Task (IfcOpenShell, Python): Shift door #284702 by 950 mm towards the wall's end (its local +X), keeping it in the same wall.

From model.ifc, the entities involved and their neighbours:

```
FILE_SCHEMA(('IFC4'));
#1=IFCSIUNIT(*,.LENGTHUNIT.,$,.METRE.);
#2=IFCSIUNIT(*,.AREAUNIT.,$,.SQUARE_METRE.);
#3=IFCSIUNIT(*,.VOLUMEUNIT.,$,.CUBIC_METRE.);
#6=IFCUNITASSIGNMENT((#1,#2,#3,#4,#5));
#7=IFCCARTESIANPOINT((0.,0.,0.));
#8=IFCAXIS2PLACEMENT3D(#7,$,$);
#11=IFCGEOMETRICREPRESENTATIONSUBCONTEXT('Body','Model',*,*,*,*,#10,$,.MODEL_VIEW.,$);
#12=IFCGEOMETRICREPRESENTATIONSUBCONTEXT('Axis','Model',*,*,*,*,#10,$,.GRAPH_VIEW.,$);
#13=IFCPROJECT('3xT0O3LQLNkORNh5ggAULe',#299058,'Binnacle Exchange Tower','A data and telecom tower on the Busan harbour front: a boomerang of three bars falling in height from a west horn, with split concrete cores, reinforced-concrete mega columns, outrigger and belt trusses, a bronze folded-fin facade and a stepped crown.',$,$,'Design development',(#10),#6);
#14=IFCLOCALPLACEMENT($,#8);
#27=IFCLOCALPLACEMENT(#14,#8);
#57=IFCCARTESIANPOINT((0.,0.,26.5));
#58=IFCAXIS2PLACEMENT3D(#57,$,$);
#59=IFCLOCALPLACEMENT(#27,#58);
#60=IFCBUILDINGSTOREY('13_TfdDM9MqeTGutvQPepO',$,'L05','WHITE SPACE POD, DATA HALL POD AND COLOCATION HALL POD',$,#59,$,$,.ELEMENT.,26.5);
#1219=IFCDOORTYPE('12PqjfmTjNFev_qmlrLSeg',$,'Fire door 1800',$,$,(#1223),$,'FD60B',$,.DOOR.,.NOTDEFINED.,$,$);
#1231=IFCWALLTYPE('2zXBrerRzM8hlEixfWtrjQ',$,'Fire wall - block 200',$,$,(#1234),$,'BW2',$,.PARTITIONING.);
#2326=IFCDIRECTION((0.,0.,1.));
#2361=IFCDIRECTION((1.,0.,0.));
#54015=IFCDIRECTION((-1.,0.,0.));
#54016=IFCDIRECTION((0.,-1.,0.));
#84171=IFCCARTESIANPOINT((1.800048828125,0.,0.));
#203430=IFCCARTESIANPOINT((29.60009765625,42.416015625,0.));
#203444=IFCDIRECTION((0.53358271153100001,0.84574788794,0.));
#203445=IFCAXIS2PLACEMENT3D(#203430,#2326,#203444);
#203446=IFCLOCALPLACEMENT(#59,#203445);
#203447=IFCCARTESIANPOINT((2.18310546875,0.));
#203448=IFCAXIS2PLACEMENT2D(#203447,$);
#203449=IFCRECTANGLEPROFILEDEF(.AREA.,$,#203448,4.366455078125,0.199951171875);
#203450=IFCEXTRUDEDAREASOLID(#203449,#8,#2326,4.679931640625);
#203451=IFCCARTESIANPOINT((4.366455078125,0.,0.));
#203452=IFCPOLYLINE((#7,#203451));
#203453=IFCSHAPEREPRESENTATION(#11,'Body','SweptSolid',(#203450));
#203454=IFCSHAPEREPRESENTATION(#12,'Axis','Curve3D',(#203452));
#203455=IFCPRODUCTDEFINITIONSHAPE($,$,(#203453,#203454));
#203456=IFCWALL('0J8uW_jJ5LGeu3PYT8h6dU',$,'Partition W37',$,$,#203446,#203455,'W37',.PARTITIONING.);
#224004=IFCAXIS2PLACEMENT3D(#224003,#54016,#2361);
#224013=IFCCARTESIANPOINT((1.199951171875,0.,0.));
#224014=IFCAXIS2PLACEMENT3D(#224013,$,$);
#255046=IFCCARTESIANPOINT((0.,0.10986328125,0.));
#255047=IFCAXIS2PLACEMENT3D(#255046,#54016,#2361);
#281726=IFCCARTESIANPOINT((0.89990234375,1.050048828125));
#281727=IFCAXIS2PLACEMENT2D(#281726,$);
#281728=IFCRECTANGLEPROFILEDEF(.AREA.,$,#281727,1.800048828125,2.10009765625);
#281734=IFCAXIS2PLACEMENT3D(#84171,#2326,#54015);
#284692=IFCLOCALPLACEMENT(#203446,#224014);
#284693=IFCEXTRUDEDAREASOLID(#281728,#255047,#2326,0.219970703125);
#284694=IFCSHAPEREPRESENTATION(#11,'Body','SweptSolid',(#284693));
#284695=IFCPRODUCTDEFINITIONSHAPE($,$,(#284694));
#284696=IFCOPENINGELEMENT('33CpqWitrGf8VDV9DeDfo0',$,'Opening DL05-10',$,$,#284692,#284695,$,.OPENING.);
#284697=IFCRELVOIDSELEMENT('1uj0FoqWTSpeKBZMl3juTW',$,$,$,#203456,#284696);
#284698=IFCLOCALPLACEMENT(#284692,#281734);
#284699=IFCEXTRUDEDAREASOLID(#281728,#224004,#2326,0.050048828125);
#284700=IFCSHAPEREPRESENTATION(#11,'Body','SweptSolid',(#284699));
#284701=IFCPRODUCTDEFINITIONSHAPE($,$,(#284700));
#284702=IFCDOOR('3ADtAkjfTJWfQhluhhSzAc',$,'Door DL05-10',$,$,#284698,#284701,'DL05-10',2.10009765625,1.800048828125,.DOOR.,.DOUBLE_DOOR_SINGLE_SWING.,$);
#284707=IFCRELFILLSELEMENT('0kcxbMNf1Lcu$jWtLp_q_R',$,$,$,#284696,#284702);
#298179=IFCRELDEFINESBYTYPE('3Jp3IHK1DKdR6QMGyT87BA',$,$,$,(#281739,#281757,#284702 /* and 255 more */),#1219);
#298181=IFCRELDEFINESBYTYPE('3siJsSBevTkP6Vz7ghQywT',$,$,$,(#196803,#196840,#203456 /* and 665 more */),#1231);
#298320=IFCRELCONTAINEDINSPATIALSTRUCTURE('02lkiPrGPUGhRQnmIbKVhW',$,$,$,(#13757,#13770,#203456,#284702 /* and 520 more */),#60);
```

```python
import ifcopenshell
import ifcopenshell.api.geometry
import ifcopenshell.util.placement
import ifcopenshell.util.unit

model = ifcopenshell.open("model.ifc")
unit_scale = ifcopenshell.util.unit.calculate_unit_scale(model)

door = model.by_guid("3ADtAkjfTJWfQhluhhSzAc")
opening = door.FillsVoids[0].RelatingOpeningElement
wall = opening.VoidsElements[0].RelatingBuildingElement

wall_matrix = ifcopenshell.util.placement.get_local_placement(wall.ObjectPlacement)
shift = wall_matrix[:3, 0] * 0.95 / unit_scale
before = ifcopenshell.util.placement.get_local_placement(door.ObjectPlacement)[:3, 3].copy()

# The door is placed relative to its opening, so it follows when the opening moves.
matrix = ifcopenshell.util.placement.get_local_placement(opening.ObjectPlacement)
matrix[:3, 3] += shift
ifcopenshell.api.geometry.edit_object_placement(
    model, product=opening, matrix=matrix, is_si=False, should_transform_children=True
)

after = ifcopenshell.util.placement.get_local_placement(door.ObjectPlacement)[:3, 3]
print("door moved by", (after - before).round(3) + 0.0)

model.write("model_edited.ifc")
```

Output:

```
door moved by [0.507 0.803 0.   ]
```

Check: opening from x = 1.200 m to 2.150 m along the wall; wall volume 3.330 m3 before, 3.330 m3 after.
